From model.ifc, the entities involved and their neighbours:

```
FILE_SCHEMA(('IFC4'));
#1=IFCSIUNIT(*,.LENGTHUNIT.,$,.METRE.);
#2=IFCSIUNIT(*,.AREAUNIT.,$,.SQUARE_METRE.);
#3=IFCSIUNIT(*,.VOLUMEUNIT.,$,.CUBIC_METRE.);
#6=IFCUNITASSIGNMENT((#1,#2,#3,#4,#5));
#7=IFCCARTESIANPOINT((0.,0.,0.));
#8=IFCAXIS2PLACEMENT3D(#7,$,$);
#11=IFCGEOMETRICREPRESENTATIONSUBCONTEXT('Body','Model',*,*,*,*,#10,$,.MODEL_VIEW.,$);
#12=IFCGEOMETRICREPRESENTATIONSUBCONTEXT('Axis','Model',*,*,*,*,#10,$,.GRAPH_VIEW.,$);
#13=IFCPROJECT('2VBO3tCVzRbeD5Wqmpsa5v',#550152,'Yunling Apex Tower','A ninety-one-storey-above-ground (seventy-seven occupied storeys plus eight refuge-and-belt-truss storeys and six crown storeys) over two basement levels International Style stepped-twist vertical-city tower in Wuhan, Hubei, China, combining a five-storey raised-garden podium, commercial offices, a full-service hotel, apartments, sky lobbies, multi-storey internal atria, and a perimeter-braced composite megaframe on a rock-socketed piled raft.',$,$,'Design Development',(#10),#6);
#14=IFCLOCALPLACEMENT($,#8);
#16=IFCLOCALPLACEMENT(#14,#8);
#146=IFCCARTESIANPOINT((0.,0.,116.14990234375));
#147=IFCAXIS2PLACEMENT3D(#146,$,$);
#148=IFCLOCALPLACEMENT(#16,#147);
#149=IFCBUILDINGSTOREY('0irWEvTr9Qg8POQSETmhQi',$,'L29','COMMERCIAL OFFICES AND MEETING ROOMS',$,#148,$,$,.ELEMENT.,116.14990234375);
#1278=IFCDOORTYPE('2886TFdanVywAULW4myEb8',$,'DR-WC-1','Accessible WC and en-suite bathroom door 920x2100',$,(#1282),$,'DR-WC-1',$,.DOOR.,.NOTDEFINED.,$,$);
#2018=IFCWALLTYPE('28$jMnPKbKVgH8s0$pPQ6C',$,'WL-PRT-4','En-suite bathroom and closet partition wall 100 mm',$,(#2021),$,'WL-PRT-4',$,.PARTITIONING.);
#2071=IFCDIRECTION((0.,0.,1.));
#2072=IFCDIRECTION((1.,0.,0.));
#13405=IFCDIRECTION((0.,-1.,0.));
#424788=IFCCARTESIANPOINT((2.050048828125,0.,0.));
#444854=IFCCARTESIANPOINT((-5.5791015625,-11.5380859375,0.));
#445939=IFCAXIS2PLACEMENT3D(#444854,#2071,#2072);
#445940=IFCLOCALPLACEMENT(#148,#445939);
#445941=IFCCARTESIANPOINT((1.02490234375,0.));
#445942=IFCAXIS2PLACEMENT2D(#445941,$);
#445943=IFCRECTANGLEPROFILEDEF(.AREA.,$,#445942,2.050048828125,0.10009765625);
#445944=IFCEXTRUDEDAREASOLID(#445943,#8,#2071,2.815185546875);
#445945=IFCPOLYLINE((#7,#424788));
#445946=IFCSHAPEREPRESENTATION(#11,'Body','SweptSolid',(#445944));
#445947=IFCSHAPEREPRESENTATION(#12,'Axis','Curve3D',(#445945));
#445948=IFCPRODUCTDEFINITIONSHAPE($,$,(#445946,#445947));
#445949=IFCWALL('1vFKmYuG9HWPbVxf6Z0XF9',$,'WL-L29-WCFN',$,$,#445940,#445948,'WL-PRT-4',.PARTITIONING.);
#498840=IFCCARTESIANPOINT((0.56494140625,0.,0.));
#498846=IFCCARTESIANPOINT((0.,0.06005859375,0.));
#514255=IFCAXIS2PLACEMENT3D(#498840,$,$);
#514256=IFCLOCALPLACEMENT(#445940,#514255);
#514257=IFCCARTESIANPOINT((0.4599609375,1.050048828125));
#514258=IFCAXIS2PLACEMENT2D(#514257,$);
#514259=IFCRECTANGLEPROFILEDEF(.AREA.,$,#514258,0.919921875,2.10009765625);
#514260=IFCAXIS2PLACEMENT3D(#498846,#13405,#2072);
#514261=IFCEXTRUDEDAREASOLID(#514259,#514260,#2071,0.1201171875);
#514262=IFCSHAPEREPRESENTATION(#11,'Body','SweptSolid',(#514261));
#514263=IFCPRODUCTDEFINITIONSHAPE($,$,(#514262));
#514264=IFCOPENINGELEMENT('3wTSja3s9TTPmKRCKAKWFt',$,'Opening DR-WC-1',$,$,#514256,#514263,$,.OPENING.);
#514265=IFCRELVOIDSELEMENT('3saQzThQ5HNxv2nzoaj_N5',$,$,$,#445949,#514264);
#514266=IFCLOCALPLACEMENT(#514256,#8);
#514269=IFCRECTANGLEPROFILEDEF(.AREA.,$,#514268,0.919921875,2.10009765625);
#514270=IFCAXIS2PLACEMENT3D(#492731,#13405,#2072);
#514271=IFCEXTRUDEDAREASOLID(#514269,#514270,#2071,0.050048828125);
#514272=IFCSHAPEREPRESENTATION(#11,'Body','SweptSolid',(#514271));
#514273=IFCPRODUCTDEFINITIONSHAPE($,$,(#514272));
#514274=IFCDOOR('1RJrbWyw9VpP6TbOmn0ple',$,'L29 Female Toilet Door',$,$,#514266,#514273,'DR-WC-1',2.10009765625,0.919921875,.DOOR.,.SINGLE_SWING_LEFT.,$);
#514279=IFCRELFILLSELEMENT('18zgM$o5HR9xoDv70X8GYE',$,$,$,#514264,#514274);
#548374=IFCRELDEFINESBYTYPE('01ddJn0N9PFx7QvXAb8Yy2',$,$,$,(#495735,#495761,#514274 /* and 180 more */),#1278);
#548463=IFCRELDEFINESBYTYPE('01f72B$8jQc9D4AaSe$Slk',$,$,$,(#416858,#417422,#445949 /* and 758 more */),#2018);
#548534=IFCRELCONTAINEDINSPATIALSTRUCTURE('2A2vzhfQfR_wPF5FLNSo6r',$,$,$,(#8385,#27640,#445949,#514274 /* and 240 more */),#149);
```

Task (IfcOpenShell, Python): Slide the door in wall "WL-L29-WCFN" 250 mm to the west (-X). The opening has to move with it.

```python
import ifcopenshell
import ifcopenshell.api.geometry
import ifcopenshell.util.placement

model = ifcopenshell.open("model.ifc")

door = model.by_guid("1RJrbWyw9VpP6TbOmn0ple")
opening = door.FillsVoids[0].RelatingOpeningElement
wall = opening.VoidsElements[0].RelatingBuildingElement

wall_matrix = ifcopenshell.util.placement.get_local_placement(wall.ObjectPlacement)
shift = wall_matrix[:3, 0] * -0.25
before = ifcopenshell.util.placement.get_local_placement(door.ObjectPlacement)[:3, 3].copy()

# The door is placed relative to its opening, so it follows when the opening moves.
matrix = ifcopenshell.util.placement.get_local_placement(opening.ObjectPlacement)
matrix[:3, 3] += shift
ifcopenshell.api.geometry.edit_object_placement(
    model, product=opening, matrix=matrix, is_si=False, should_transform_children=True
)

after = ifcopenshell.util.placement.get_local_placement(door.ObjectPlacement)[:3, 3]
print("door moved by", (after - before).round(3) + 0.0)

model.write("model-out.ifc")
```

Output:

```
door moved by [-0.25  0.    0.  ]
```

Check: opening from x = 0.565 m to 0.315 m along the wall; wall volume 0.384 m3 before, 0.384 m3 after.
